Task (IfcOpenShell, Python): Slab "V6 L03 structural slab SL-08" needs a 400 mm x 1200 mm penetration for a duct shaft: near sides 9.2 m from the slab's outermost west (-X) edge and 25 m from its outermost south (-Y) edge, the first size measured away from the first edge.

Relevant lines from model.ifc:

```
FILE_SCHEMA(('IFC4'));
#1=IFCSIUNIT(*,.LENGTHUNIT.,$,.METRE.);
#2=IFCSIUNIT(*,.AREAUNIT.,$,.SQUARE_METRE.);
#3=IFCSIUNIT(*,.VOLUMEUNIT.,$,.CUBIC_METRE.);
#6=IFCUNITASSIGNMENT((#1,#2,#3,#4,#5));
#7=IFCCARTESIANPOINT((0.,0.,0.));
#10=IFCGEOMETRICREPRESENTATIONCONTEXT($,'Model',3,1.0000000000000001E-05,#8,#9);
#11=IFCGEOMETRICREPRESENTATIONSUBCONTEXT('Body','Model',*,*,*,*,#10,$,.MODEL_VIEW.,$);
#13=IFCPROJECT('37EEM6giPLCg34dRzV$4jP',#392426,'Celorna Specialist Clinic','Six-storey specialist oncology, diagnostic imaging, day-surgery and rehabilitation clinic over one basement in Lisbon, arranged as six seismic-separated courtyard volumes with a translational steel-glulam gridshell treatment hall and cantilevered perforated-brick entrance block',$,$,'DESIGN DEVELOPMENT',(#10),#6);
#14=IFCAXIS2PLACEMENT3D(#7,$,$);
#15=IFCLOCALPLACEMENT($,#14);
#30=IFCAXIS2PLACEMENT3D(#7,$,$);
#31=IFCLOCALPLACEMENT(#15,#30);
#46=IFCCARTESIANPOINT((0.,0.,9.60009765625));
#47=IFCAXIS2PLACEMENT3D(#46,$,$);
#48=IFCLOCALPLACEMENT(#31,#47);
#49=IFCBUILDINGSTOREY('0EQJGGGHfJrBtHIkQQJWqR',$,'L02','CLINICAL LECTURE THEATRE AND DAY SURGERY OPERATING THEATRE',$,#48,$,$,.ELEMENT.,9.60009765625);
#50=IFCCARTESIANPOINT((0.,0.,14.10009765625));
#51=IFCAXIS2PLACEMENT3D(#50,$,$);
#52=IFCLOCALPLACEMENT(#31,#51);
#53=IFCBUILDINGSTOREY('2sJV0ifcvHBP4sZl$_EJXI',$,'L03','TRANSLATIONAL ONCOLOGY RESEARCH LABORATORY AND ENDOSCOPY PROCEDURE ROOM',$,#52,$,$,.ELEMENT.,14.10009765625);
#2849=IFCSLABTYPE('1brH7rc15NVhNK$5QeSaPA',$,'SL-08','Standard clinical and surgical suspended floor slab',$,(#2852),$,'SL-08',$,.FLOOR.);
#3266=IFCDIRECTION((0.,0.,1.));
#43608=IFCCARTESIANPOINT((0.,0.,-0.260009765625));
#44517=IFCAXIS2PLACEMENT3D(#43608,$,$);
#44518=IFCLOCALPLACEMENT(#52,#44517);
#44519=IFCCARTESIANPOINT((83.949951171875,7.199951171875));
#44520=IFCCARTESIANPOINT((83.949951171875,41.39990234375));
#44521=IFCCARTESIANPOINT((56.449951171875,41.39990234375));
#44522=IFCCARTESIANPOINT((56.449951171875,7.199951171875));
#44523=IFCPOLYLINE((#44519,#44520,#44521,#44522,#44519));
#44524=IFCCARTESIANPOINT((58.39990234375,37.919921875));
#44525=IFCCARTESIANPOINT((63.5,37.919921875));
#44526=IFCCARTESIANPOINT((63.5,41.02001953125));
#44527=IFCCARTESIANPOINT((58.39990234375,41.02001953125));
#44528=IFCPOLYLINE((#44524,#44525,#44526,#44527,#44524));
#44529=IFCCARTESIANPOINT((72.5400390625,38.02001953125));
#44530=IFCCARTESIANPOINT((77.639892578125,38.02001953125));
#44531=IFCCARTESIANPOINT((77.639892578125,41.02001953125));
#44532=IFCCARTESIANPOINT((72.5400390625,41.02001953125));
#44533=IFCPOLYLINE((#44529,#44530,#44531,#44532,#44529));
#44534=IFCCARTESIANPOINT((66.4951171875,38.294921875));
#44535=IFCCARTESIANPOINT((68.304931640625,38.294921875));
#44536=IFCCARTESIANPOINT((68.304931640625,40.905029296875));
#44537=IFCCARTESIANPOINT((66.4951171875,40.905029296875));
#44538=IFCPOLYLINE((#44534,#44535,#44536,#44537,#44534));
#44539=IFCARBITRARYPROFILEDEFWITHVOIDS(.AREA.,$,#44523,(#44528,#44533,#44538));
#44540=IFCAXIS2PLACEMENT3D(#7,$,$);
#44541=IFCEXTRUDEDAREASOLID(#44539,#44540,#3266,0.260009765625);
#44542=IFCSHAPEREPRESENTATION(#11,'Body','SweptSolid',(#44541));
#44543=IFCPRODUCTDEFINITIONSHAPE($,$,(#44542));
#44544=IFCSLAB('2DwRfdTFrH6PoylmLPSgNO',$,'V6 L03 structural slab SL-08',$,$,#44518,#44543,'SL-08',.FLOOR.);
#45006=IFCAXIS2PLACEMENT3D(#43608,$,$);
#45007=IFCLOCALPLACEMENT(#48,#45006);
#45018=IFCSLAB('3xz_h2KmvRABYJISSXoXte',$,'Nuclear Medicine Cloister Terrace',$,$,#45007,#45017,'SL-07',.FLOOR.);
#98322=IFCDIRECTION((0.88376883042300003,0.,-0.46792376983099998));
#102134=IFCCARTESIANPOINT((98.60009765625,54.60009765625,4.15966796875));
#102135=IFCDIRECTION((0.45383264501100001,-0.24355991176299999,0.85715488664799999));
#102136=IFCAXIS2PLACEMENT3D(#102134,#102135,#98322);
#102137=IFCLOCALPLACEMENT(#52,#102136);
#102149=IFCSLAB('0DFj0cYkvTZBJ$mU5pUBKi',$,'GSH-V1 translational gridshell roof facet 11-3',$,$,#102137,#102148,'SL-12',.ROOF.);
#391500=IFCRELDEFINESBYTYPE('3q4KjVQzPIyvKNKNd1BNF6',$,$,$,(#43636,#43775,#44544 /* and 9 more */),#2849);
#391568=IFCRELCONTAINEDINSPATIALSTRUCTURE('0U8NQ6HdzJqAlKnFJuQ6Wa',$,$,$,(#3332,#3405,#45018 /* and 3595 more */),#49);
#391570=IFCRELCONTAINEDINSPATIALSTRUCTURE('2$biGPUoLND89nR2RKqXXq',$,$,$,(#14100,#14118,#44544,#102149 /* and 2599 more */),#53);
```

```python
import numpy as np
import ifcopenshell
import ifcopenshell.api.feature
import ifcopenshell.api.geometry
import ifcopenshell.api.root
import ifcopenshell.geom
import ifcopenshell.util.placement
import ifcopenshell.util.representation
import ifcopenshell.util.shape
import ifcopenshell.util.unit

model = ifcopenshell.open("model.ifc")
unit_scale = ifcopenshell.util.unit.calculate_unit_scale(model)
settings = ifcopenshell.geom.settings()


def volume(element):
    """Net volume in cubic metres, openings subtracted."""
    shape = ifcopenshell.geom.create_shape(settings, element)
    return ifcopenshell.util.shape.get_volume(shape.geometry)


slab = model.by_id(44544)
before = volume(slab)

# Extent in the slab's own axes, in metres. The edges named are its -X and -Y sides.
slab_shape = ifcopenshell.geom.create_shape(settings, slab)
vertices = ifcopenshell.util.shape.get_vertices(slab_shape.geometry)
x_min, y_min, bottom = vertices.min(axis=0)
top = vertices[:, 2].max()

opening = ifcopenshell.api.root.create_entity(model, ifc_class="IfcOpeningElement", name="Duct shaft opening", predefined_type="OPENING")
context = ifcopenshell.util.representation.get_context(model, "Model", "Body", "MODEL_VIEW")
width, depth = 0.4, 1.2
outline = [(0.0, 0.0), (width, 0.0), (width, depth), (0.0, depth), (0.0, 0.0)]
# Overshoot both faces by 50 mm so the cut is clean.
shape = ifcopenshell.api.geometry.add_slab_representation(
    model, context=context, depth=top - bottom + 0.1, polyline=outline
)
ifcopenshell.api.geometry.assign_representation(model, product=opening, representation=shape)

matrix = ifcopenshell.util.placement.get_local_placement(slab.ObjectPlacement)
matrix[:, 3] = matrix @ np.append(np.array([x_min + 9.2, y_min + 25, bottom - 0.05]) / unit_scale, 1.0)
ifcopenshell.api.geometry.edit_object_placement(model, product=opening, matrix=matrix, is_si=False)
ifcopenshell.api.feature.add_feature(model, feature=opening, element=slab)

after = volume(slab)

print(f"slab volume {before:.3f} -> {after:.3f} m3")

model.write("model-out.ifc")
```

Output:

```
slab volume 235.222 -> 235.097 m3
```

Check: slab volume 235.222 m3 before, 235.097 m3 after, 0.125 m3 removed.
